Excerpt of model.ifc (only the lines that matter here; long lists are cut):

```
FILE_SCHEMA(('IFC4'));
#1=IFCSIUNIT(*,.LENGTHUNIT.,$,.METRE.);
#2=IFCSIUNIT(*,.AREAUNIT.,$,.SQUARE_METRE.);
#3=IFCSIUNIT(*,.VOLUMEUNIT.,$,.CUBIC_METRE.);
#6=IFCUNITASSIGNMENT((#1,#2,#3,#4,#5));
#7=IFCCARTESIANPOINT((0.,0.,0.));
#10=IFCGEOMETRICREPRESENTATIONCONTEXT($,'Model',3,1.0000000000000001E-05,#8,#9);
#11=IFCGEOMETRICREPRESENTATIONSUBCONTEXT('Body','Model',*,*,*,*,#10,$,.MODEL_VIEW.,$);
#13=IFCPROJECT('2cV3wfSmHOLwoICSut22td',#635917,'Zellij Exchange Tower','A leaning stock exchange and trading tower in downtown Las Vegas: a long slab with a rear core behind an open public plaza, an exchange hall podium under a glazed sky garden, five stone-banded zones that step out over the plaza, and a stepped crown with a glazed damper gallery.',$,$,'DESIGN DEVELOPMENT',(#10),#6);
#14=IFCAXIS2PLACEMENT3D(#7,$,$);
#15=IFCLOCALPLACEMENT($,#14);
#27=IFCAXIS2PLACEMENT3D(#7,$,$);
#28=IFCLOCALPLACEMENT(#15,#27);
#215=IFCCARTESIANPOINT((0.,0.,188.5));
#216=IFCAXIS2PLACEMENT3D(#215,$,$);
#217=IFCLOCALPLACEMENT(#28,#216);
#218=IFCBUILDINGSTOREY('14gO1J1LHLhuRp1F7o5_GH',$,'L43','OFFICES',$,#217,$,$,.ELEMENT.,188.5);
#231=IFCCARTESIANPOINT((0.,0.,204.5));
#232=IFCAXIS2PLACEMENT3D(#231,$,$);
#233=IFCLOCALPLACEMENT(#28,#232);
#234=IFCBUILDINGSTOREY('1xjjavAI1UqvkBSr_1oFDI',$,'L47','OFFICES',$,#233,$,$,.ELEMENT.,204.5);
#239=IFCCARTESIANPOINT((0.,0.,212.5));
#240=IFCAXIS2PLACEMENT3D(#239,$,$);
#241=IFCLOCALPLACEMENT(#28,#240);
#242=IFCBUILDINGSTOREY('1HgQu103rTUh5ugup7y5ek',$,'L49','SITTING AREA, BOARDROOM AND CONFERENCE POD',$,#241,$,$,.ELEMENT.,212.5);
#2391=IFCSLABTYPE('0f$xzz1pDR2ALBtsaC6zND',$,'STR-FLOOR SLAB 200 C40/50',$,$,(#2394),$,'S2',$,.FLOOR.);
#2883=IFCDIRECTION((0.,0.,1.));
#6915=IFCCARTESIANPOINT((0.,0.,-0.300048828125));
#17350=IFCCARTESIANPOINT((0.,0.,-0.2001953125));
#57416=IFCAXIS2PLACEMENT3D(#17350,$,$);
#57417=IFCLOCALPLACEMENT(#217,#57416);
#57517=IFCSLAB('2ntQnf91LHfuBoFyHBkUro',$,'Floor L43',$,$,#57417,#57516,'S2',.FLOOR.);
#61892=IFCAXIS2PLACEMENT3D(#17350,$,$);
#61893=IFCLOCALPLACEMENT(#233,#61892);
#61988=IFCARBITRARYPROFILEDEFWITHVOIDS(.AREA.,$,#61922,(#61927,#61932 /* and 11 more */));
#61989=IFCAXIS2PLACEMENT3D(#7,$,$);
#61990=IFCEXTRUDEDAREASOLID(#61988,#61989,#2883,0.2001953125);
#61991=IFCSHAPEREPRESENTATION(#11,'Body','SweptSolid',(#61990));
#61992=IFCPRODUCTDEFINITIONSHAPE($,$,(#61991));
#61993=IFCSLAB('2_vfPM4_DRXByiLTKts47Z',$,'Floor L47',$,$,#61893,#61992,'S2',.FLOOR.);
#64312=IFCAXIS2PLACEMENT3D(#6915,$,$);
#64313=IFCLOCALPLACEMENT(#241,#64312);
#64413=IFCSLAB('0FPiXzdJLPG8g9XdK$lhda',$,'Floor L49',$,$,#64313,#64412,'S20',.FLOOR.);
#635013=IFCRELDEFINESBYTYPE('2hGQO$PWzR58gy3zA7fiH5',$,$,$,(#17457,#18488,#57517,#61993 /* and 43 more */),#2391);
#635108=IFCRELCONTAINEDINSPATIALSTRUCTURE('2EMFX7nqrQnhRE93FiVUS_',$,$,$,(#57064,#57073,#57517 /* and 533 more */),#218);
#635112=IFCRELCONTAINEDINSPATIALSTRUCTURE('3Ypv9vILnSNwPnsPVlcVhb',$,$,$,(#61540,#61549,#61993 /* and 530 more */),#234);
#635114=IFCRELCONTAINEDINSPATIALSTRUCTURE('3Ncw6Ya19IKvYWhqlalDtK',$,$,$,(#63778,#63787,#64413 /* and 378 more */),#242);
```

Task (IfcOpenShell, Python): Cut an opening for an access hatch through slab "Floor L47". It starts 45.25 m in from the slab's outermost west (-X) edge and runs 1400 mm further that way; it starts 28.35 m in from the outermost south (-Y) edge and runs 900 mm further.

```python
import numpy as np
import ifcopenshell
import ifcopenshell.api.feature
import ifcopenshell.api.geometry
import ifcopenshell.api.root
import ifcopenshell.geom
import ifcopenshell.util.placement
import ifcopenshell.util.representation
import ifcopenshell.util.shape
import ifcopenshell.util.unit

model = ifcopenshell.open("model.ifc")
unit_scale = ifcopenshell.util.unit.calculate_unit_scale(model)
settings = ifcopenshell.geom.settings()


def volume(element):
    """Net volume in cubic metres, openings subtracted."""
    shape = ifcopenshell.geom.create_shape(settings, element)
    return ifcopenshell.util.shape.get_volume(shape.geometry)


slab = model.by_guid("2_vfPM4_DRXByiLTKts47Z")
before = volume(slab)

# Extent in the slab's own axes, in metres. The edges named are its -X and -Y sides.
slab_shape = ifcopenshell.geom.create_shape(settings, slab)
vertices = ifcopenshell.util.shape.get_vertices(slab_shape.geometry)
x_min, y_min, bottom = vertices.min(axis=0)
top = vertices[:, 2].max()

opening = ifcopenshell.api.root.create_entity(model, ifc_class="IfcOpeningElement", name="Access hatch opening", predefined_type="OPENING")
context = ifcopenshell.util.representation.get_context(model, "Model", "Body", "MODEL_VIEW")
width, depth = 1.4, 0.9
outline = [(0.0, 0.0), (width, 0.0), (width, depth), (0.0, depth), (0.0, 0.0)]
# Overshoot both faces by 50 mm so the cut is clean.
shape = ifcopenshell.api.geometry.add_slab_representation(
    model, context=context, depth=top - bottom + 0.1, polyline=outline
)
ifcopenshell.api.geometry.assign_representation(model, product=opening, representation=shape)

matrix = ifcopenshell.util.placement.get_local_placement(slab.ObjectPlacement)
matrix[:, 3] = matrix @ np.append(np.array([x_min + 45.25, y_min + 28.35, bottom - 0.05]) / unit_scale, 1.0)
ifcopenshell.api.geometry.edit_object_placement(model, product=opening, matrix=matrix, is_si=False)
ifcopenshell.api.feature.add_feature(model, feature=opening, element=slab)

after = volume(slab)

print(f"slab volume {before:.3f} -> {after:.3f} m3")

model.write("model_rev.ifc")
```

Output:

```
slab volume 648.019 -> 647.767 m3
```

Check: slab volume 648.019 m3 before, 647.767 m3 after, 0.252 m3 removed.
